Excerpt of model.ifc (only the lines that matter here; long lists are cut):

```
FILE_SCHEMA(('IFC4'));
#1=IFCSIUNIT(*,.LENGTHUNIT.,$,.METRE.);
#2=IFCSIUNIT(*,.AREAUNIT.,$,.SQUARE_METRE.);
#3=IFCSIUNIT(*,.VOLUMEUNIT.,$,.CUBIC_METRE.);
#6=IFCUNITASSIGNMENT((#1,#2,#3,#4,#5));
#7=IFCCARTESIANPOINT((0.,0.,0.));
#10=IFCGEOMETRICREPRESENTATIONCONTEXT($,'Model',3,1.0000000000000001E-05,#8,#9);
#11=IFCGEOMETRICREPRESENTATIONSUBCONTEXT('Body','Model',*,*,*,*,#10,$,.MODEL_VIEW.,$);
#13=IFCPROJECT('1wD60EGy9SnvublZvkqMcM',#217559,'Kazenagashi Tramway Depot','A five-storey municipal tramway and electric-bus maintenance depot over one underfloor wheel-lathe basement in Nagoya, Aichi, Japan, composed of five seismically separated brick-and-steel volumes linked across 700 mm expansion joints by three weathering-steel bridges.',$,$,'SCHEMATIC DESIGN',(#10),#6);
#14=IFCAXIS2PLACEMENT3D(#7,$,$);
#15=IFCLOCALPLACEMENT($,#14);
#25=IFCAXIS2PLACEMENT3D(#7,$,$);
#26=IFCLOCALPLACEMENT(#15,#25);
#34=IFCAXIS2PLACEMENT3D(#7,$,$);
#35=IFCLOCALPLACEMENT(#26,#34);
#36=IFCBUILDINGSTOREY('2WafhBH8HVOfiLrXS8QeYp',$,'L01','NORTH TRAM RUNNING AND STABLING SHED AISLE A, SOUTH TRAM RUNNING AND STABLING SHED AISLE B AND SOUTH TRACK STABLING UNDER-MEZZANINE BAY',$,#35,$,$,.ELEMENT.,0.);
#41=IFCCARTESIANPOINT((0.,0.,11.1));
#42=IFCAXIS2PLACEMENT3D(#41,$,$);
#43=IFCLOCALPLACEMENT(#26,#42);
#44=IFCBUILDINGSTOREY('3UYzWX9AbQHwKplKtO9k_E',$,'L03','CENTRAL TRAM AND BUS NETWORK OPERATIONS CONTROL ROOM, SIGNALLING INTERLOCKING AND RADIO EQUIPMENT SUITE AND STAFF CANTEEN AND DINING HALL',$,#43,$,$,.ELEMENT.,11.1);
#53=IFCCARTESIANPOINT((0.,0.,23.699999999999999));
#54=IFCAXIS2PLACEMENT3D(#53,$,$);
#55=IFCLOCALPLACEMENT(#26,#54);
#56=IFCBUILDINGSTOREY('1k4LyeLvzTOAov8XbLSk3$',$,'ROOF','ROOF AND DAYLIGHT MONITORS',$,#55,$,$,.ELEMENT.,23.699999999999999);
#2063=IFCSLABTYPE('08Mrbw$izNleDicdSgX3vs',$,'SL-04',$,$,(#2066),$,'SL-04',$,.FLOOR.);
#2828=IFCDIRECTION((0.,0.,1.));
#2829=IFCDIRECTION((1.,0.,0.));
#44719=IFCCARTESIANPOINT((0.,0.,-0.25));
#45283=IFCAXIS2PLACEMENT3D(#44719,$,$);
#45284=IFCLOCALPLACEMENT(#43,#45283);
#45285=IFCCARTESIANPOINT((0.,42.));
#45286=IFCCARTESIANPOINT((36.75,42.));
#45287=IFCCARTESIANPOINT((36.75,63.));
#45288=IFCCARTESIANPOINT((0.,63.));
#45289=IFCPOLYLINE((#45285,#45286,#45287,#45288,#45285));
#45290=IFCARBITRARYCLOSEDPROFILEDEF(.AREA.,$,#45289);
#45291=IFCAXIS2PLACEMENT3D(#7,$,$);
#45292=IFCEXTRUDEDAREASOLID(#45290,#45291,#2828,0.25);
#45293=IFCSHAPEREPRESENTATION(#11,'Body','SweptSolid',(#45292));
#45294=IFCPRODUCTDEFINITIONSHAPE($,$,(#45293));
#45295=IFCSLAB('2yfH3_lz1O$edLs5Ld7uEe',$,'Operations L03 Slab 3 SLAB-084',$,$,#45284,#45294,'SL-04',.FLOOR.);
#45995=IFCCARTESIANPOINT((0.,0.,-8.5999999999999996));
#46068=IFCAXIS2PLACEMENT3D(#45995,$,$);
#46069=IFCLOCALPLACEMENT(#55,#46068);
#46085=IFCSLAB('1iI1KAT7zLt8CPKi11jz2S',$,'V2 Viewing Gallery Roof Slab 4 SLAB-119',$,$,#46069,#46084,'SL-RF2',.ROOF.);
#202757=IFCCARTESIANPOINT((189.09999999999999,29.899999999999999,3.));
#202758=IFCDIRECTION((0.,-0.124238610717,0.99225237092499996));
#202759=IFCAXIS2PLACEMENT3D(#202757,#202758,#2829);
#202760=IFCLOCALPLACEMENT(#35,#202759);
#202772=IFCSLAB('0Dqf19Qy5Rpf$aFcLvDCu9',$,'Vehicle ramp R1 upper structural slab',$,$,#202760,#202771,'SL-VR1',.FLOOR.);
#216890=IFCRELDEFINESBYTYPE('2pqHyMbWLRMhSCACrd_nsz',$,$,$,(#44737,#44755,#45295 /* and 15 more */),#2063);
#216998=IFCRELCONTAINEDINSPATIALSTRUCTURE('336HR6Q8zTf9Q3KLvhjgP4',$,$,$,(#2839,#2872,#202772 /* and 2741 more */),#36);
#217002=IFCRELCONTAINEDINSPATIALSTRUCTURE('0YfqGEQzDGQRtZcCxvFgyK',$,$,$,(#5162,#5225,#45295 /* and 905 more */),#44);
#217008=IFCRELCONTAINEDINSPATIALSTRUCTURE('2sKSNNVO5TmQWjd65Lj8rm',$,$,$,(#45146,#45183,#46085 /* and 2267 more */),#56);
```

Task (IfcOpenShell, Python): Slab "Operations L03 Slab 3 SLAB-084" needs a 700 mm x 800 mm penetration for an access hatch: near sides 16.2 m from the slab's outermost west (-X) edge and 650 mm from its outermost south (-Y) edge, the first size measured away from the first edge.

```python
import numpy as np
import ifcopenshell
import ifcopenshell.api.feature
import ifcopenshell.api.geometry
import ifcopenshell.api.root
import ifcopenshell.geom
import ifcopenshell.util.placement
import ifcopenshell.util.representation
import ifcopenshell.util.shape
import ifcopenshell.util.unit

model = ifcopenshell.open("model.ifc")
unit_scale = ifcopenshell.util.unit.calculate_unit_scale(model)
settings = ifcopenshell.geom.settings()


def volume(element):
    """Net volume in cubic metres, openings subtracted."""
    shape = ifcopenshell.geom.create_shape(settings, element)
    return ifcopenshell.util.shape.get_volume(shape.geometry)


slab = model.by_id(45295)
before = volume(slab)

# Extent in the slab's own axes, in metres. The edges named are its -X and -Y sides.
slab_shape = ifcopenshell.geom.create_shape(settings, slab)
vertices = ifcopenshell.util.shape.get_vertices(slab_shape.geometry)
x_min, y_min, bottom = vertices.min(axis=0)
top = vertices[:, 2].max()

opening = ifcopenshell.api.root.create_entity(model, ifc_class="IfcOpeningElement", name="Access hatch opening", predefined_type="OPENING")
context = ifcopenshell.util.representation.get_context(model, "Model", "Body", "MODEL_VIEW")
width, depth = 0.7, 0.8
outline = [(0.0, 0.0), (width, 0.0), (width, depth), (0.0, depth), (0.0, 0.0)]
# Overshoot both faces by 50 mm so the cut is clean.
shape = ifcopenshell.api.geometry.add_slab_representation(
    model, context=context, depth=top - bottom + 0.1, polyline=outline
)
ifcopenshell.api.geometry.assign_representation(model, product=opening, representation=shape)

matrix = ifcopenshell.util.placement.get_local_placement(slab.ObjectPlacement)
matrix[:, 3] = matrix @ np.append(np.array([x_min + 16.2, y_min + 0.65, bottom - 0.05]) / unit_scale, 1.0)
ifcopenshell.api.geometry.edit_object_placement(model, product=opening, matrix=matrix, is_si=False)
ifcopenshell.api.feature.add_feature(model, feature=opening, element=slab)

after = volume(slab)

print(f"slab volume {before:.3f} -> {after:.3f} m3")

model.write("model_v2.ifc")
```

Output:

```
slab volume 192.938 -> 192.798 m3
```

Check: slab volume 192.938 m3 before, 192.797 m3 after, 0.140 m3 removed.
